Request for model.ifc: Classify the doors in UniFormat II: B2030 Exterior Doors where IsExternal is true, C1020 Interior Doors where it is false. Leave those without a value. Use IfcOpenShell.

First a look at what the model holds.

```python
import ifcopenshell
import ifcopenshell.util.element

model = ifcopenshell.open("model.ifc")
print(model.schema)
print("classifications:", [c.Name for c in model.by_type("IfcClassification")])
values = [ifcopenshell.util.element.get_pset(e, "Pset_DoorCommon", "IsExternal") for e in model.by_type("IfcDoor")]
for value in (True, False, None):
    print("IsExternal", value, values.count(value))
```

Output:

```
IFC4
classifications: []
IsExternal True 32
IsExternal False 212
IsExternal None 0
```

```python
import ifcopenshell
import ifcopenshell.api.classification
import ifcopenshell.util.element

model = ifcopenshell.open("model.ifc")

system = ifcopenshell.api.classification.add_classification(model, classification="UniFormat II")

doors = model.by_type("IfcDoor")
external = {e: ifcopenshell.util.element.get_pset(e, "Pset_DoorCommon", "IsExternal") for e in doors}
for flag, code, name in ((True, "B2030", "Exterior Doors"), (False, "C1020", "Interior Doors")):
    products = [e for e in doors if external[e] is flag]
    ifcopenshell.api.classification.add_reference(
        model, products=products, classification=system, identification=code, name=name
    )
    print(code, len(products))

model.write("model_v2.ifc")
```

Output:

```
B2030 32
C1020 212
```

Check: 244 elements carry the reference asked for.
